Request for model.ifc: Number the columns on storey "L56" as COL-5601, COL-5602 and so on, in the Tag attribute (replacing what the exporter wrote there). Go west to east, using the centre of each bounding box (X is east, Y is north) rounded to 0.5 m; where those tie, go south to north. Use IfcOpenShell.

First a look at what the model holds.

```python
import ifcopenshell
import ifcopenshell.util.element
import ifcopenshell.util.placement

model = ifcopenshell.open("model.ifc")
print(model.schema)
storey = next(s for s in model.by_type("IfcBuildingStorey") if s.Name == "L56")
columns = [e for e in ifcopenshell.util.element.get_decomposition(storey) if e.is_a("IfcColumn")]
for e in sorted(columns, key=lambda e: e.id()):
    origin = ifcopenshell.util.placement.get_local_placement(e.ObjectPlacement)[:3, 3]
    print(e.id(), e.Tag, e.Name, origin.round(2) + 0.0, sep=" | ")
```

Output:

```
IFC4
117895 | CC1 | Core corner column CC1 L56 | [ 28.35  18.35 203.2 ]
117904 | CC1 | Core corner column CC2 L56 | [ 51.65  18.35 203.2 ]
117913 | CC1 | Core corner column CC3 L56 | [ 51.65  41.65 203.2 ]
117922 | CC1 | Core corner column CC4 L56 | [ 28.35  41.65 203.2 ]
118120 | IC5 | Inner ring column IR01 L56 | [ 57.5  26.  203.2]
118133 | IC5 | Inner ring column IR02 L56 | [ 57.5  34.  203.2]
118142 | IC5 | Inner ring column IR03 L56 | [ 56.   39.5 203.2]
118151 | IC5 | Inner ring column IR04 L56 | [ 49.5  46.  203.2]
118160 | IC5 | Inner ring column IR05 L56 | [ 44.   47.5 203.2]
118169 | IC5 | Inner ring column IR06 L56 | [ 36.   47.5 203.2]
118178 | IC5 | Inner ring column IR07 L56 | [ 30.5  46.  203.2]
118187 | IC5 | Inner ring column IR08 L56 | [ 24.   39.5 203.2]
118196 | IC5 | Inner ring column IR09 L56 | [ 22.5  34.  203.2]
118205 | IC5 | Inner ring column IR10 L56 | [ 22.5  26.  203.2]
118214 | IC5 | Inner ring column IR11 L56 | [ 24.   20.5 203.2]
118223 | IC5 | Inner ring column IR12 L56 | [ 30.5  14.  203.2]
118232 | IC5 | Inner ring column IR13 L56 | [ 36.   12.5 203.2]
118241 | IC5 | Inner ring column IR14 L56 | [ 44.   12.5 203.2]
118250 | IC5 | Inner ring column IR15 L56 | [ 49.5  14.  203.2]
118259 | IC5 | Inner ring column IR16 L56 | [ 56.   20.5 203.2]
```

```python
import ifcopenshell
import ifcopenshell.geom
import ifcopenshell.util.element
import ifcopenshell.util.shape

model = ifcopenshell.open("model.ifc")
settings = ifcopenshell.geom.settings()
settings.set("use-world-coords", True)


def centre(element):
    shape = ifcopenshell.geom.create_shape(settings, element)
    return ifcopenshell.util.shape.get_bbox_centroid(shape.geometry)


storey = next(s for s in model.by_type("IfcBuildingStorey") if s.Name == "L56")
columns = [e for e in ifcopenshell.util.element.get_decomposition(storey) if e.is_a("IfcColumn")]

# Insertion points can sit at a corner or the storey origin, so sort by the geometry (in metres).
centres = {e: centre(e) for e in columns}
columns.sort(key=lambda e: (round(centres[e][0] / 0.5), centres[e][1]))

for i, e in enumerate(columns, start=1):
    number = f"COL-56{i:02d}"
    e.Tag = number
    print(e.id(), number)

model.write("model-out.ifc")
```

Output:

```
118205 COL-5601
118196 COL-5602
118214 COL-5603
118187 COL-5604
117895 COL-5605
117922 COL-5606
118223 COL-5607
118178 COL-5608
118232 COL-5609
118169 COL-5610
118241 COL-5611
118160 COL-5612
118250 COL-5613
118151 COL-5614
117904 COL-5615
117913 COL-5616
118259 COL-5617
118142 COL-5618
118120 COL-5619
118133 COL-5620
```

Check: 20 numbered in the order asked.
